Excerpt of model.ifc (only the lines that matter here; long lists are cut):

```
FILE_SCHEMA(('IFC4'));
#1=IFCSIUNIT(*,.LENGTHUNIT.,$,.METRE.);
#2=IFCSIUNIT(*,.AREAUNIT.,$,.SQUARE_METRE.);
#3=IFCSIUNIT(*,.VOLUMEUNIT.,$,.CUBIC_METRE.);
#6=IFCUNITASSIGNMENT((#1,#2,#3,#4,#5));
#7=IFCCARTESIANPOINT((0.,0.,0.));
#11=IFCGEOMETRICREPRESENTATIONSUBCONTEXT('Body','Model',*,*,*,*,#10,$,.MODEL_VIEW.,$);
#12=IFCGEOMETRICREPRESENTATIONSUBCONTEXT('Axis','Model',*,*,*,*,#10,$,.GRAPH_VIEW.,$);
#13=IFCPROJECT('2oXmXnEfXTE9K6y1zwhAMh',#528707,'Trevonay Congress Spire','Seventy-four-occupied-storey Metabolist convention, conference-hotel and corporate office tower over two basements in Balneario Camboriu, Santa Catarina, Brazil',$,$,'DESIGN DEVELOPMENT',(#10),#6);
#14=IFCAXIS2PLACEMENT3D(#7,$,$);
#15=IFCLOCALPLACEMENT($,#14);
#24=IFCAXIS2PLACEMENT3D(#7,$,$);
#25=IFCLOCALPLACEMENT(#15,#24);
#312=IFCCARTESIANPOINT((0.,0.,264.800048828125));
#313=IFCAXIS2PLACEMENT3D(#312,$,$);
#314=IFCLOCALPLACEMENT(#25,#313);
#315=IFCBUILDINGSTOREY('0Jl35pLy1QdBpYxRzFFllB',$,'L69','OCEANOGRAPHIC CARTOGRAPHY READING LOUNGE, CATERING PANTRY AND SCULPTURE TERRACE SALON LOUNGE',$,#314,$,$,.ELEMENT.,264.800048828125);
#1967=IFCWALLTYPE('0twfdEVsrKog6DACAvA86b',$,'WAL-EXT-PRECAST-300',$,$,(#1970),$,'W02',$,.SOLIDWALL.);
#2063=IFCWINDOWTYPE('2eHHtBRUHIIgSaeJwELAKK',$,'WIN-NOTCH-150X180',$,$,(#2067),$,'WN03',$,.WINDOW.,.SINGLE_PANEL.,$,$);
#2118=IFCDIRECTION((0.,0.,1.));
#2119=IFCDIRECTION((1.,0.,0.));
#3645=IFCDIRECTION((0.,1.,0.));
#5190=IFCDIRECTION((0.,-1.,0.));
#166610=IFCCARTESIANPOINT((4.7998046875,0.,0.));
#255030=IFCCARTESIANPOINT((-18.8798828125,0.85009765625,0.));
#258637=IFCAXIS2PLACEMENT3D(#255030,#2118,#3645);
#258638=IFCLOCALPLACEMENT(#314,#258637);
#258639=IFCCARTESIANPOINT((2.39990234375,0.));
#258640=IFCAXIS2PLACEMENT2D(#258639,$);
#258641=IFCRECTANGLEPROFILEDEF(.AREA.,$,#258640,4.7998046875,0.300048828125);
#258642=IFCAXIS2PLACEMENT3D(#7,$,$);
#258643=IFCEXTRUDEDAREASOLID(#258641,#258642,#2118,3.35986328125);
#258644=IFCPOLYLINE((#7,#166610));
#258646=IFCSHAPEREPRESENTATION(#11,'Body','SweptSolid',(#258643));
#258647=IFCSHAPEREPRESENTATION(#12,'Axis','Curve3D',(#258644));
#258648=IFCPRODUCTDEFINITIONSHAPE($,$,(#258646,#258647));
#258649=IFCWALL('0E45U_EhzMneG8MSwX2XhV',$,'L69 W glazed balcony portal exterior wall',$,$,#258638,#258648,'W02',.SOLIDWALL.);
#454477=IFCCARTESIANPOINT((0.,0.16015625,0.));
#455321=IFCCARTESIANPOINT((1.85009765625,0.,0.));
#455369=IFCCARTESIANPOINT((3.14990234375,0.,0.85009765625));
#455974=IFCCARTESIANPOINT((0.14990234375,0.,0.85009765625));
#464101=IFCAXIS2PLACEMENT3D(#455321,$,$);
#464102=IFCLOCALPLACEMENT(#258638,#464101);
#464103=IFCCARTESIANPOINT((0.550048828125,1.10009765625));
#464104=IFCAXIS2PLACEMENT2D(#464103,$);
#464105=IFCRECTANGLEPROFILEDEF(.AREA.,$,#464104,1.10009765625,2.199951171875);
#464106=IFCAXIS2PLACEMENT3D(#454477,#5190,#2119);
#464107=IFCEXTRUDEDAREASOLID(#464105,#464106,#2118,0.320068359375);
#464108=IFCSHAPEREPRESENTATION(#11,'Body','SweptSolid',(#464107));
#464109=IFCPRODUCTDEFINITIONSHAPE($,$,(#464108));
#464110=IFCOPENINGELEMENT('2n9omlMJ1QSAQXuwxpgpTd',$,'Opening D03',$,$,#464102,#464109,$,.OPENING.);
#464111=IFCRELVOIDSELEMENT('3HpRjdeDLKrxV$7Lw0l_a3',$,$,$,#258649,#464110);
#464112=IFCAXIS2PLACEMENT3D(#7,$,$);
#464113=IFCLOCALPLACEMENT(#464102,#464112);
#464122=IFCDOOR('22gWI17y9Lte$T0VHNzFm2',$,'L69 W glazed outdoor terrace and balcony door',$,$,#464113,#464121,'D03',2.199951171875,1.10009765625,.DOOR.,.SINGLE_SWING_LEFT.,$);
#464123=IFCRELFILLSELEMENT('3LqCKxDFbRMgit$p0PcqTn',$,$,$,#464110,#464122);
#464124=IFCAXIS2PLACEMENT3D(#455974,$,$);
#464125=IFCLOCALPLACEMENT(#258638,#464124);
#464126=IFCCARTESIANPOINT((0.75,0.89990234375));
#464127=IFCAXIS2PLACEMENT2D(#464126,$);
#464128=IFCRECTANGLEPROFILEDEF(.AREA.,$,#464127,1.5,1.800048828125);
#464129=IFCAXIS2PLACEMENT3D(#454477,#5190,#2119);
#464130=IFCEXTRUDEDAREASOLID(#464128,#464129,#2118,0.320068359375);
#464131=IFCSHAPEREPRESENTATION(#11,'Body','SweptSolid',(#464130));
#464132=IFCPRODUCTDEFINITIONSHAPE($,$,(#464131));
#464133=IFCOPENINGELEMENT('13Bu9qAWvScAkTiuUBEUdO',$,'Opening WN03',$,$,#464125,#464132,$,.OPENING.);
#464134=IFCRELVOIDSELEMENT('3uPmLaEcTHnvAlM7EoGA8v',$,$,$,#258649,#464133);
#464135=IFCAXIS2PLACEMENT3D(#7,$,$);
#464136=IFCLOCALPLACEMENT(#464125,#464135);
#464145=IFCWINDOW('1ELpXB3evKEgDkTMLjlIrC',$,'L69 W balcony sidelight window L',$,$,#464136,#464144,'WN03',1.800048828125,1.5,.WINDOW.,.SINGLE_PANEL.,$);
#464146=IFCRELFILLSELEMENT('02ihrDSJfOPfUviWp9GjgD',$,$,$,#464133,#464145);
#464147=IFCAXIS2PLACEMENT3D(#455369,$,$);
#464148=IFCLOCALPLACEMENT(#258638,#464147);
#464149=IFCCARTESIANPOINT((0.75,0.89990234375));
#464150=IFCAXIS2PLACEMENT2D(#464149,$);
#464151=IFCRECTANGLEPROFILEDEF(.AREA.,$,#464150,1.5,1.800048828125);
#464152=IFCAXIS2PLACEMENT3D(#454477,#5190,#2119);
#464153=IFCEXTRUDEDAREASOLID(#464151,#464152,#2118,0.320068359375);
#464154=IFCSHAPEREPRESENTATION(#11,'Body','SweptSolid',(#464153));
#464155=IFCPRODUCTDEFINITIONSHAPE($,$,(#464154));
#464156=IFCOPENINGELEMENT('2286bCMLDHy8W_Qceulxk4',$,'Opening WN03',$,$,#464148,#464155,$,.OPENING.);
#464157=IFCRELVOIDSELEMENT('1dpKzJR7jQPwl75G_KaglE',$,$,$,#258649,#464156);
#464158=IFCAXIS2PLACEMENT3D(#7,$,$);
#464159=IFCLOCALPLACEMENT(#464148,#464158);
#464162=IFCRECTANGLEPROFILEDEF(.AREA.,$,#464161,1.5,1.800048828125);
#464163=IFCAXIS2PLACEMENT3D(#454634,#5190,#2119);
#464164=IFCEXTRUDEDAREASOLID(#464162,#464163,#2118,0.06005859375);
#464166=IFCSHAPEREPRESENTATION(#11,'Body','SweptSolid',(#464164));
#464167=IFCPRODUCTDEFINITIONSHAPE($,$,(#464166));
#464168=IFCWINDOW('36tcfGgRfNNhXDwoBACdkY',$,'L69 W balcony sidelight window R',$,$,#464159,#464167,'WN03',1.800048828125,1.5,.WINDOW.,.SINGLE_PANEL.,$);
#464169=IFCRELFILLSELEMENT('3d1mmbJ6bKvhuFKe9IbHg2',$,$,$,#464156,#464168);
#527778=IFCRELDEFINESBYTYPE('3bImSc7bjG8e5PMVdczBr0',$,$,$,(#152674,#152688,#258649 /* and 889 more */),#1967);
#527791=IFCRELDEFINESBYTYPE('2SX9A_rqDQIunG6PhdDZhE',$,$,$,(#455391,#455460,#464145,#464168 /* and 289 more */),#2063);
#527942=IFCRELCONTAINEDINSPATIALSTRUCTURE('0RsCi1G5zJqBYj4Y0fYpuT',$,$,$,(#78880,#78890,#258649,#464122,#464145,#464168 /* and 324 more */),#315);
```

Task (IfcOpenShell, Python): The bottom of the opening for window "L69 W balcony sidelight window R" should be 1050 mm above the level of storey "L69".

```python
import numpy as np
import ifcopenshell
import ifcopenshell.api.geometry
import ifcopenshell.geom
import ifcopenshell.util.element
import ifcopenshell.util.placement
import ifcopenshell.util.shape
import ifcopenshell.util.unit

model = ifcopenshell.open("model.ifc")
unit_scale = ifcopenshell.util.unit.calculate_unit_scale(model)

window = model.by_id(464168)
opening = window.FillsVoids[0].RelatingOpeningElement
storey = ifcopenshell.util.element.get_container(window, ifc_class="IfcBuildingStorey")
level = ifcopenshell.util.placement.get_local_placement(storey.ObjectPlacement)[2, 3]

# The opening's origin need not be at the sill, so measure its lowest point.
shape = ifcopenshell.geom.create_shape(ifcopenshell.geom.settings(), opening)
bottom = ifcopenshell.util.shape.get_shape_bottom_elevation(shape, shape.geometry) / unit_scale
dz = level + 1.05 / unit_scale - bottom

shift = np.array([0.0, 0.0, dz])
# The window is placed relative to its opening, so it follows when the opening moves.
matrix = ifcopenshell.util.placement.get_local_placement(opening.ObjectPlacement)
matrix[:3, 3] += shift
ifcopenshell.api.geometry.edit_object_placement(
    model, product=opening, matrix=matrix, is_si=False, should_transform_children=True
)

print(f"moved by {dz * unit_scale:+.3f} m")

model.write("model_updated.ifc")
```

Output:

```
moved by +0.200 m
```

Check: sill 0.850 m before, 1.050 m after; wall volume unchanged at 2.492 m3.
